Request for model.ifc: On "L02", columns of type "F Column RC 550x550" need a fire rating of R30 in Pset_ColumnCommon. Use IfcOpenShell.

First a look at what the model holds.

```python
import ifcopenshell
import ifcopenshell.util.element

model = ifcopenshell.open("model.ifc")
print(model.schema)
storey = next(s for s in model.by_type("IfcBuildingStorey") if s.Name == "L02")
columns = [e for e in ifcopenshell.util.element.get_decomposition(storey) if e.is_a("IfcColumn")]
seen = {}
for e in columns:
    element_type = ifcopenshell.util.element.get_type(e)
    key = (element_type.Name if element_type != e and element_type else None, ifcopenshell.util.element.get_pset(e, "Pset_ColumnCommon", "FireRating"))
    seen[key] = seen.get(key, 0) + 1
for (name, value), count in sorted(seen.items(), key=str):
    print(count, "x", name, "|", value)
```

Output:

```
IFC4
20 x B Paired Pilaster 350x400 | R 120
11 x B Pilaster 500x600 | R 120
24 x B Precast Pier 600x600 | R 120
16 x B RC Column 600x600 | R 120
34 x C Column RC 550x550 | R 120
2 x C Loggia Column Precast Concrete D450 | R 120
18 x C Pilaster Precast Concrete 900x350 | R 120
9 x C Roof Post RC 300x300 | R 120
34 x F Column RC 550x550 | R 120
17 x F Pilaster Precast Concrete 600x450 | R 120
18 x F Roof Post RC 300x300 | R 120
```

```python
import ifcopenshell
import ifcopenshell.api.pset
import ifcopenshell.util.element

model = ifcopenshell.open("model.ifc")

storey = next(s for s in model.by_type("IfcBuildingStorey") if s.Name == "L02")
columns = [e for e in ifcopenshell.util.element.get_decomposition(storey) if e.is_a("IfcColumn")]

count = 0
for e in columns:
    element_type = ifcopenshell.util.element.get_type(e)
    if element_type in (None, e) or element_type.Name != "F Column RC 550x550":
        continue
    # add_pset returns the element's existing set when there is one.
    pset = ifcopenshell.api.pset.add_pset(model, product=e, name="Pset_ColumnCommon")
    ifcopenshell.api.pset.edit_pset(model, pset=pset, properties={"FireRating": "R30"})
    count += 1

print(count, "columns updated")

model.write("model-out.ifc")
```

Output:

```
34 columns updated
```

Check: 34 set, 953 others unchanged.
